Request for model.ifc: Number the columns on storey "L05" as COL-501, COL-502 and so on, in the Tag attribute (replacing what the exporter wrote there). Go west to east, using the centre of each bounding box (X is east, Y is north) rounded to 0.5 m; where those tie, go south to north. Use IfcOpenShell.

First a look at what the model holds.

```python
import ifcopenshell
import ifcopenshell.util.element
import ifcopenshell.util.placement

model = ifcopenshell.open("model.ifc")
print(model.schema)
storey = next(s for s in model.by_type("IfcBuildingStorey") if s.Name == "L05")
columns = [e for e in ifcopenshell.util.element.get_decomposition(storey) if e.is_a("IfcColumn")]
for e in sorted(columns, key=lambda e: e.id()):
    origin = ifcopenshell.util.placement.get_local_placement(e.ObjectPlacement)[:3, 3]
    print(e.id(), e.Tag, e.Name, origin.round(2) + 0.0, sep=" | ")
```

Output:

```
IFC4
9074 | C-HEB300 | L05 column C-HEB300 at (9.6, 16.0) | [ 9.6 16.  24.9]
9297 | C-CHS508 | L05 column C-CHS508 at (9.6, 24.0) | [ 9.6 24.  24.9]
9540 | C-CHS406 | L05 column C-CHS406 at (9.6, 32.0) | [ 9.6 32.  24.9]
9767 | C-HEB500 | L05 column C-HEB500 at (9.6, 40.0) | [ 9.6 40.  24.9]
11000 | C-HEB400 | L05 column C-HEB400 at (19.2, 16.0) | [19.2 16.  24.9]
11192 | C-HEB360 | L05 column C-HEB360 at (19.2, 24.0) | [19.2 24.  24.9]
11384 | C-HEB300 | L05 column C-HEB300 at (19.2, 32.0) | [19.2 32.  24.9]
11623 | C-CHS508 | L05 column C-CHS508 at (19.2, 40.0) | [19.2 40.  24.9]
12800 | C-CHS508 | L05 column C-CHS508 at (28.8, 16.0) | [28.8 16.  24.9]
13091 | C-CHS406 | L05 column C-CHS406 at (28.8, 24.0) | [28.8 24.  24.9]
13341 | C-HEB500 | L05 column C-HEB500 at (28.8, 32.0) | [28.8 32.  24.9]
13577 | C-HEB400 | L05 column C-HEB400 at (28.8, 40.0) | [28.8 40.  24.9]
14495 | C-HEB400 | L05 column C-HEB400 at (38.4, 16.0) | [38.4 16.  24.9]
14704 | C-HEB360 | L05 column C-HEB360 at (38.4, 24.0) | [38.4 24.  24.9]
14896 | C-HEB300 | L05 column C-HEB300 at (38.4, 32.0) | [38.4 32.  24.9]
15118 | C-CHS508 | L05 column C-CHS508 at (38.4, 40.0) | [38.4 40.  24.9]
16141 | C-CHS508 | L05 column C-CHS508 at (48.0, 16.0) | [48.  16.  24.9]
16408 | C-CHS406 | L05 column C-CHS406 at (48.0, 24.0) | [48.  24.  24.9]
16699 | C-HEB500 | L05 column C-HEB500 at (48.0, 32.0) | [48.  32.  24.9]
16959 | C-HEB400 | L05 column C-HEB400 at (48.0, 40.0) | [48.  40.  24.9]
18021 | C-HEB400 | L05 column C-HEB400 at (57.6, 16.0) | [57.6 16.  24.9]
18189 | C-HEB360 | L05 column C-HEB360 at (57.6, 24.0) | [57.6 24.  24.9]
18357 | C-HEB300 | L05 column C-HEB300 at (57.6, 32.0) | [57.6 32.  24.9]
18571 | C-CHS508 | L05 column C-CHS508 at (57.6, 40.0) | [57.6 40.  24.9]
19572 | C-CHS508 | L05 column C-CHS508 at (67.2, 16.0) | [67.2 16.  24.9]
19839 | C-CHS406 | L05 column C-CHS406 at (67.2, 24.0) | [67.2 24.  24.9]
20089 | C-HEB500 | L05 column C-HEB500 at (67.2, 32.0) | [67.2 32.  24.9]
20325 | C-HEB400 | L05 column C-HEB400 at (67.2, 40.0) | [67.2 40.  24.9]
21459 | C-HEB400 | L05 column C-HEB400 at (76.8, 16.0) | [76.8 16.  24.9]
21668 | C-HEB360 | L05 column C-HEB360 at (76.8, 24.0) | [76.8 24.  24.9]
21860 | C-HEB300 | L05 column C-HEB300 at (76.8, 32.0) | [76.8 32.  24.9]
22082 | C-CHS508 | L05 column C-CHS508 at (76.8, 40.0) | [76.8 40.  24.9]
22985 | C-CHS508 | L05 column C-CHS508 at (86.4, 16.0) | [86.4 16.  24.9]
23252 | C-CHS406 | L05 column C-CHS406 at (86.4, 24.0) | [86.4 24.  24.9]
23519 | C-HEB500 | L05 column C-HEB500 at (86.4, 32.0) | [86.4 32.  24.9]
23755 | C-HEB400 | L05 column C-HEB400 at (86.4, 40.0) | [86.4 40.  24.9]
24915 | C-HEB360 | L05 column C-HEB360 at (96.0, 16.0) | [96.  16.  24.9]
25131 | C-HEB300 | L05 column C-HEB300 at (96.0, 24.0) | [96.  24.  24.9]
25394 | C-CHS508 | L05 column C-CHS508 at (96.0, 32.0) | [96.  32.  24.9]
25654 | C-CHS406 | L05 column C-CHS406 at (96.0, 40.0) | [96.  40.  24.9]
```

```python
import ifcopenshell
import ifcopenshell.geom
import ifcopenshell.util.element
import ifcopenshell.util.shape

model = ifcopenshell.open("model.ifc")
settings = ifcopenshell.geom.settings()
settings.set("use-world-coords", True)


def centre(element):
    shape = ifcopenshell.geom.create_shape(settings, element)
    return ifcopenshell.util.shape.get_bbox_centroid(shape.geometry)


storey = next(s for s in model.by_type("IfcBuildingStorey") if s.Name == "L05")
columns = [e for e in ifcopenshell.util.element.get_decomposition(storey) if e.is_a("IfcColumn")]

# Insertion points can sit at a corner or the storey origin, so sort by the geometry (in metres).
centres = {e: centre(e) for e in columns}
columns.sort(key=lambda e: (round(centres[e][0] / 0.5), centres[e][1]))

for i, e in enumerate(columns, start=1):
    number = f"COL-5{i:02d}"
    e.Tag = number
    print(e.id(), number)

model.write("model_rev.ifc")
```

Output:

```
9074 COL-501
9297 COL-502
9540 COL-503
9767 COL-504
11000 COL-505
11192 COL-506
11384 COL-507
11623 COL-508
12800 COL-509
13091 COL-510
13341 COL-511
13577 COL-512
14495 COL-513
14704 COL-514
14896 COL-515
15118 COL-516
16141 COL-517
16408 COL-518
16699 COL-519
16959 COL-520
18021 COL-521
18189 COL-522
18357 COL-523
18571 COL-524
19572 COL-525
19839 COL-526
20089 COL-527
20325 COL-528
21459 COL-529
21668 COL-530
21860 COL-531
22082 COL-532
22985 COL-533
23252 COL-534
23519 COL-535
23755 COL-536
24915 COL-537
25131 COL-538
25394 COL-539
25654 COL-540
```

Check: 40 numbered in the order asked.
